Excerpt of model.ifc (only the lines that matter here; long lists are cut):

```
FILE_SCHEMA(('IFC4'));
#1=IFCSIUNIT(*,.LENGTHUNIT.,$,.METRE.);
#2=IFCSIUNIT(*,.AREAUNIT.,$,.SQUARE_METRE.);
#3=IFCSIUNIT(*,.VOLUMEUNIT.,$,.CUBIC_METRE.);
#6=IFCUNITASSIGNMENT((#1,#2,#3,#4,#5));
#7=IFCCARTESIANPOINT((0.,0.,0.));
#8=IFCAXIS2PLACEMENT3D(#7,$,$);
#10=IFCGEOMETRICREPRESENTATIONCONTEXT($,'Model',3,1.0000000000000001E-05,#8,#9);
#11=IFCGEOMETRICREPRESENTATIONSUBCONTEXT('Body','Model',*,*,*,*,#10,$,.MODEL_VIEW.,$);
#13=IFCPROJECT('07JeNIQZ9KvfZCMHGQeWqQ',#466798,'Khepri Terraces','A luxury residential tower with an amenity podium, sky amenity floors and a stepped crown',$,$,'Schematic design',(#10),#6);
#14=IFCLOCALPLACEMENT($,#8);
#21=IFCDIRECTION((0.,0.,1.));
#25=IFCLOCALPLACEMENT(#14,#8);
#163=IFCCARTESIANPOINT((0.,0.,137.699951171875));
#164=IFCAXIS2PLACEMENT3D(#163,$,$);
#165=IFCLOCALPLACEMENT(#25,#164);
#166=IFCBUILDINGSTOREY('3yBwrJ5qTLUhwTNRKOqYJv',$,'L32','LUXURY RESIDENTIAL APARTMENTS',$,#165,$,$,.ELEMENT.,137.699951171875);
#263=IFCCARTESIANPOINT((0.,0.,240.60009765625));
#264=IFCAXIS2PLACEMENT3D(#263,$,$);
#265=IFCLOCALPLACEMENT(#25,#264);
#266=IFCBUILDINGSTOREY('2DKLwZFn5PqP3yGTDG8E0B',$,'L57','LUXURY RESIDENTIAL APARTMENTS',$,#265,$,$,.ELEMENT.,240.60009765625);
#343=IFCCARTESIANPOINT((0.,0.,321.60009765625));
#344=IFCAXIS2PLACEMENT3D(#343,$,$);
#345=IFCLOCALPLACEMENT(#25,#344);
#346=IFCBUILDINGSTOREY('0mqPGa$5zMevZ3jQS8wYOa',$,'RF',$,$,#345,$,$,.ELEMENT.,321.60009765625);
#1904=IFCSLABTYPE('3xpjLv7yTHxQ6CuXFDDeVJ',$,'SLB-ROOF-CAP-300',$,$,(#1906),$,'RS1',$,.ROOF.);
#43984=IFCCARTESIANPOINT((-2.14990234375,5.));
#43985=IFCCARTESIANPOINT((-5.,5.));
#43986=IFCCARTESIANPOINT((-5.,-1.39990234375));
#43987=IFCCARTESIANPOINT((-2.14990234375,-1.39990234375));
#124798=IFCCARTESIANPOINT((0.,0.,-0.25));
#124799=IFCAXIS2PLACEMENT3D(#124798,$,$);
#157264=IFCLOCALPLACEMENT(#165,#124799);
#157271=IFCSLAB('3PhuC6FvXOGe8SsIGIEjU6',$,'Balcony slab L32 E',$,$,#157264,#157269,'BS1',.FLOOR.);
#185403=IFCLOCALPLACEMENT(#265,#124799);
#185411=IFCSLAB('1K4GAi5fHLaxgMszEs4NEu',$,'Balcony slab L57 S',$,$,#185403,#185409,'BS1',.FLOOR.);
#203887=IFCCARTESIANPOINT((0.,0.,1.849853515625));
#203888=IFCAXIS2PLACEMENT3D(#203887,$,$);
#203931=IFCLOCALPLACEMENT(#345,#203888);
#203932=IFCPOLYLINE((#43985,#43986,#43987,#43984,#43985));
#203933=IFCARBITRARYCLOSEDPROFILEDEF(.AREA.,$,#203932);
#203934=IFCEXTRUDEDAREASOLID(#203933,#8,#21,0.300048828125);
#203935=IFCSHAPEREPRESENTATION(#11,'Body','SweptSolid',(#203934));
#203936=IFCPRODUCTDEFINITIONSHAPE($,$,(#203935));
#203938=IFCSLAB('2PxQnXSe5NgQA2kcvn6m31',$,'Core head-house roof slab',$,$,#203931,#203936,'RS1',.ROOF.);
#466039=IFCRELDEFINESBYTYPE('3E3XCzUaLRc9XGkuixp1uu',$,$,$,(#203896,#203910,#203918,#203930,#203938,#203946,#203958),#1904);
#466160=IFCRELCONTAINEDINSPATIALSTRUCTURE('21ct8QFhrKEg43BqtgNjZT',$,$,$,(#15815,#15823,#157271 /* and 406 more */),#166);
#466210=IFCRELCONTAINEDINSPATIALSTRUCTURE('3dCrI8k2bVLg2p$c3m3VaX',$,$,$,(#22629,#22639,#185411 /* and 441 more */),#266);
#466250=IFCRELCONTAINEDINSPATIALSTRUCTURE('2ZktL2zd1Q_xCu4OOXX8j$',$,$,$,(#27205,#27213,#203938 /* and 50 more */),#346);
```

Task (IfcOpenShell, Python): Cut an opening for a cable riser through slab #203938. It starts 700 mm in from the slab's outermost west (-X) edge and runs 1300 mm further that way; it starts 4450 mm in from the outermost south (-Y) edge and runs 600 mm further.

```python
import numpy as np
import ifcopenshell
import ifcopenshell.api.feature
import ifcopenshell.api.geometry
import ifcopenshell.api.root
import ifcopenshell.geom
import ifcopenshell.util.placement
import ifcopenshell.util.representation
import ifcopenshell.util.shape
import ifcopenshell.util.unit

model = ifcopenshell.open("model.ifc")
unit_scale = ifcopenshell.util.unit.calculate_unit_scale(model)
settings = ifcopenshell.geom.settings()


def volume(element):
    """Net volume in cubic metres, openings subtracted."""
    shape = ifcopenshell.geom.create_shape(settings, element)
    return ifcopenshell.util.shape.get_volume(shape.geometry)


slab = model.by_guid("2PxQnXSe5NgQA2kcvn6m31")
before = volume(slab)

# Extent in the slab's own axes, in metres. The edges named are its -X and -Y sides.
slab_shape = ifcopenshell.geom.create_shape(settings, slab)
vertices = ifcopenshell.util.shape.get_vertices(slab_shape.geometry)
x_min, y_min, bottom = vertices.min(axis=0)
top = vertices[:, 2].max()

opening = ifcopenshell.api.root.create_entity(model, ifc_class="IfcOpeningElement", name="Cable riser opening", predefined_type="OPENING")
context = ifcopenshell.util.representation.get_context(model, "Model", "Body", "MODEL_VIEW")
width, depth = 1.3, 0.6
outline = [(0.0, 0.0), (width, 0.0), (width, depth), (0.0, depth), (0.0, 0.0)]
# Overshoot both faces by 50 mm so the cut is clean.
shape = ifcopenshell.api.geometry.add_slab_representation(
    model, context=context, depth=top - bottom + 0.1, polyline=outline
)
ifcopenshell.api.geometry.assign_representation(model, product=opening, representation=shape)

matrix = ifcopenshell.util.placement.get_local_placement(slab.ObjectPlacement)
matrix[:, 3] = matrix @ np.append(np.array([x_min + 0.7, y_min + 4.45, bottom - 0.05]) / unit_scale, 1.0)
ifcopenshell.api.geometry.edit_object_placement(model, product=opening, matrix=matrix, is_si=False)
ifcopenshell.api.feature.add_feature(model, feature=opening, element=slab)

after = volume(slab)

print(f"slab volume {before:.3f} -> {after:.3f} m3")

model.write("model-out.ifc")
```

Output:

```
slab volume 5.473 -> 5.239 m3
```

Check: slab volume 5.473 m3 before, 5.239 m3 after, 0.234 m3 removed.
